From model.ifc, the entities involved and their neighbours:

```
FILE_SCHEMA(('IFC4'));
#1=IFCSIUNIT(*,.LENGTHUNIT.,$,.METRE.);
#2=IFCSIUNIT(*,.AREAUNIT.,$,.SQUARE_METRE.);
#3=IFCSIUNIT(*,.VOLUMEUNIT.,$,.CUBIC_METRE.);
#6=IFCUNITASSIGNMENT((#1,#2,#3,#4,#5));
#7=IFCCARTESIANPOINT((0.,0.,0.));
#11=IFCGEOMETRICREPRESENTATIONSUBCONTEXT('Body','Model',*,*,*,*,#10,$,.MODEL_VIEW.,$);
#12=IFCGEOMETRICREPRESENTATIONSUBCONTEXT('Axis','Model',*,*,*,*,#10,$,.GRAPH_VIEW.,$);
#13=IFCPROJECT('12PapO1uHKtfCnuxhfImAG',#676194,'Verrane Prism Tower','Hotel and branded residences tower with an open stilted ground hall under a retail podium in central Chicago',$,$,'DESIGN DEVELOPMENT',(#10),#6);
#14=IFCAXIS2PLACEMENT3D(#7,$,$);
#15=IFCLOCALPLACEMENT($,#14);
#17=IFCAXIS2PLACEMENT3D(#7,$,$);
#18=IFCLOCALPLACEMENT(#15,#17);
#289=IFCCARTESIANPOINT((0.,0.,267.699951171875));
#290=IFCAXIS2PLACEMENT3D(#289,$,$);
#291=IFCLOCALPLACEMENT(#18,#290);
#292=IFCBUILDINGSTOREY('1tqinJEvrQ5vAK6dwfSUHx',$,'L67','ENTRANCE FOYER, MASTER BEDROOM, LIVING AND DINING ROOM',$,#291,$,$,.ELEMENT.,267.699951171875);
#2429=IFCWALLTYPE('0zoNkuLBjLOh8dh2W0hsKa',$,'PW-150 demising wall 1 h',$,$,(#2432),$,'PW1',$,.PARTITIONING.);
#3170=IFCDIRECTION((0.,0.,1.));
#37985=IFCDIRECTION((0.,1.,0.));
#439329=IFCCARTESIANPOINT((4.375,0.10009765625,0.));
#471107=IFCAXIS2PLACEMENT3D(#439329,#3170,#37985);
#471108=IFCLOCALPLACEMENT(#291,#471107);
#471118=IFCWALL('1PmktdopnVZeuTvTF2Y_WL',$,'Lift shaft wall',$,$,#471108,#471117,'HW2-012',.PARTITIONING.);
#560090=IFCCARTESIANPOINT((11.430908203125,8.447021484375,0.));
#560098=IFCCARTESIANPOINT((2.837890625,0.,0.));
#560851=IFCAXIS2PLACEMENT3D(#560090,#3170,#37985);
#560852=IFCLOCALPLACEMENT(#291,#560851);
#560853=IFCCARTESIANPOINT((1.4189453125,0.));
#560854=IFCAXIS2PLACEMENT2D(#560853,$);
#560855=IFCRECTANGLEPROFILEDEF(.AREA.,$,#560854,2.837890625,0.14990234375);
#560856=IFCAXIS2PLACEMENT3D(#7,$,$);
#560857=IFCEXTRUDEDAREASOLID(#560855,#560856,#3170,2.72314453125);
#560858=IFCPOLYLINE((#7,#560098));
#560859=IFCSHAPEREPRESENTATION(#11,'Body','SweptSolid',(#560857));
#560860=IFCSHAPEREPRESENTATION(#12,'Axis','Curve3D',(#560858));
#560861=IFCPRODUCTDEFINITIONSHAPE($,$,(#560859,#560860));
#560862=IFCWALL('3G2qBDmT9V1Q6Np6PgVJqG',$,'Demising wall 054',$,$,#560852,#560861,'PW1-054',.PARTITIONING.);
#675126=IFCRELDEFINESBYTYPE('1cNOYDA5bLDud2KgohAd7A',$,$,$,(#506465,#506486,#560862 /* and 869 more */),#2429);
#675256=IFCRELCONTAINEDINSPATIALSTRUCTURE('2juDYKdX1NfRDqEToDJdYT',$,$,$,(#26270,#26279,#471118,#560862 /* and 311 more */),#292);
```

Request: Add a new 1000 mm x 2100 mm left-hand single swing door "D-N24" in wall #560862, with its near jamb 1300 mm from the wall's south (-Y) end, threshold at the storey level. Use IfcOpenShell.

```python
import numpy as np
import ifcopenshell
import ifcopenshell.api.feature
import ifcopenshell.api.geometry
import ifcopenshell.api.root
import ifcopenshell.api.spatial
import ifcopenshell.geom
import ifcopenshell.util.element
import ifcopenshell.util.placement
import ifcopenshell.util.representation
import ifcopenshell.util.shape
import ifcopenshell.util.unit

model = ifcopenshell.open("model.ifc")
unit_scale = ifcopenshell.util.unit.calculate_unit_scale(model)
settings = ifcopenshell.geom.settings()


def volume(element):
    """Net volume in cubic metres, openings subtracted."""
    shape = ifcopenshell.geom.create_shape(settings, element)
    return ifcopenshell.util.shape.get_volume(shape.geometry)


wall = model.by_id(560862)
storey = ifcopenshell.util.element.get_container(wall, ifc_class="IfcBuildingStorey")
context = ifcopenshell.util.representation.get_context(model, "Model", "Body", "MODEL_VIEW")
before = volume(wall)

width, height, from_end, sill = 1, 2.1, 1.3, 0.0  # metres

# The wall runs along its own X axis, and the end named is its -X end.
wall_shape = ifcopenshell.geom.create_shape(settings, wall)
x, y, z = ifcopenshell.util.shape.get_vertices(wall_shape.geometry).T
start = x.min() + from_end
face, thickness = float(y.min()), float(y.max() - y.min())
wall_matrix = ifcopenshell.util.placement.get_local_placement(wall.ObjectPlacement)
level = ifcopenshell.util.placement.get_local_placement(storey.ObjectPlacement)[2, 3]


def in_wall(x, y):
    """Placement at x, y metres in the wall's axes, at sill height."""
    matrix = wall_matrix.copy()
    matrix[:, 3] = wall_matrix @ np.array([x / unit_scale, y / unit_scale, 0.0, 1.0])
    matrix[2, 3] = level + sill / unit_scale
    return matrix


# Opening: a box that overshoots both wall faces by 50 mm.
opening = ifcopenshell.api.root.create_entity(model, ifc_class="IfcOpeningElement", predefined_type="OPENING")
box = ifcopenshell.api.geometry.add_wall_representation(
    model, context=context, length=width, height=height, thickness=thickness + 0.1
)
ifcopenshell.api.geometry.assign_representation(model, product=opening, representation=box)
ifcopenshell.api.geometry.edit_object_placement(model, product=opening, matrix=in_wall(start, face - 0.05), is_si=False)
ifcopenshell.api.feature.add_feature(model, feature=opening, element=wall)

door = ifcopenshell.api.root.create_entity(model, ifc_class="IfcDoor", name="D-N24", predefined_type="DOOR")
door.OverallWidth, door.OverallHeight = width / unit_scale, height / unit_scale
door.OperationType = "SINGLE_SWING_LEFT"
body = ifcopenshell.api.geometry.add_door_representation(
    model,
    context=context,
    overall_width=door.OverallWidth,
    overall_height=door.OverallHeight,
    operation_type="SINGLE_SWING_LEFT",
    lining_properties={"LiningDepth": thickness / unit_scale, "ThresholdDepth": thickness / unit_scale},
)
ifcopenshell.api.geometry.assign_representation(model, product=door, representation=body)
ifcopenshell.api.spatial.assign_container(model, products=[door], relating_structure=storey)
ifcopenshell.api.feature.add_filling(model, opening=opening, element=door)

# The lining spans the wall, so the door starts at the wall face.
ifcopenshell.api.geometry.edit_object_placement(model, product=door, matrix=in_wall(start, face), is_si=False)

after = volume(wall)

print(f"wall volume {before:.3f} -> {after:.3f} m3")

model.write("model-out.ifc")
```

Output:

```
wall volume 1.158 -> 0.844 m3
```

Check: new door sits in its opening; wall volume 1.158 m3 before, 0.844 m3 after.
